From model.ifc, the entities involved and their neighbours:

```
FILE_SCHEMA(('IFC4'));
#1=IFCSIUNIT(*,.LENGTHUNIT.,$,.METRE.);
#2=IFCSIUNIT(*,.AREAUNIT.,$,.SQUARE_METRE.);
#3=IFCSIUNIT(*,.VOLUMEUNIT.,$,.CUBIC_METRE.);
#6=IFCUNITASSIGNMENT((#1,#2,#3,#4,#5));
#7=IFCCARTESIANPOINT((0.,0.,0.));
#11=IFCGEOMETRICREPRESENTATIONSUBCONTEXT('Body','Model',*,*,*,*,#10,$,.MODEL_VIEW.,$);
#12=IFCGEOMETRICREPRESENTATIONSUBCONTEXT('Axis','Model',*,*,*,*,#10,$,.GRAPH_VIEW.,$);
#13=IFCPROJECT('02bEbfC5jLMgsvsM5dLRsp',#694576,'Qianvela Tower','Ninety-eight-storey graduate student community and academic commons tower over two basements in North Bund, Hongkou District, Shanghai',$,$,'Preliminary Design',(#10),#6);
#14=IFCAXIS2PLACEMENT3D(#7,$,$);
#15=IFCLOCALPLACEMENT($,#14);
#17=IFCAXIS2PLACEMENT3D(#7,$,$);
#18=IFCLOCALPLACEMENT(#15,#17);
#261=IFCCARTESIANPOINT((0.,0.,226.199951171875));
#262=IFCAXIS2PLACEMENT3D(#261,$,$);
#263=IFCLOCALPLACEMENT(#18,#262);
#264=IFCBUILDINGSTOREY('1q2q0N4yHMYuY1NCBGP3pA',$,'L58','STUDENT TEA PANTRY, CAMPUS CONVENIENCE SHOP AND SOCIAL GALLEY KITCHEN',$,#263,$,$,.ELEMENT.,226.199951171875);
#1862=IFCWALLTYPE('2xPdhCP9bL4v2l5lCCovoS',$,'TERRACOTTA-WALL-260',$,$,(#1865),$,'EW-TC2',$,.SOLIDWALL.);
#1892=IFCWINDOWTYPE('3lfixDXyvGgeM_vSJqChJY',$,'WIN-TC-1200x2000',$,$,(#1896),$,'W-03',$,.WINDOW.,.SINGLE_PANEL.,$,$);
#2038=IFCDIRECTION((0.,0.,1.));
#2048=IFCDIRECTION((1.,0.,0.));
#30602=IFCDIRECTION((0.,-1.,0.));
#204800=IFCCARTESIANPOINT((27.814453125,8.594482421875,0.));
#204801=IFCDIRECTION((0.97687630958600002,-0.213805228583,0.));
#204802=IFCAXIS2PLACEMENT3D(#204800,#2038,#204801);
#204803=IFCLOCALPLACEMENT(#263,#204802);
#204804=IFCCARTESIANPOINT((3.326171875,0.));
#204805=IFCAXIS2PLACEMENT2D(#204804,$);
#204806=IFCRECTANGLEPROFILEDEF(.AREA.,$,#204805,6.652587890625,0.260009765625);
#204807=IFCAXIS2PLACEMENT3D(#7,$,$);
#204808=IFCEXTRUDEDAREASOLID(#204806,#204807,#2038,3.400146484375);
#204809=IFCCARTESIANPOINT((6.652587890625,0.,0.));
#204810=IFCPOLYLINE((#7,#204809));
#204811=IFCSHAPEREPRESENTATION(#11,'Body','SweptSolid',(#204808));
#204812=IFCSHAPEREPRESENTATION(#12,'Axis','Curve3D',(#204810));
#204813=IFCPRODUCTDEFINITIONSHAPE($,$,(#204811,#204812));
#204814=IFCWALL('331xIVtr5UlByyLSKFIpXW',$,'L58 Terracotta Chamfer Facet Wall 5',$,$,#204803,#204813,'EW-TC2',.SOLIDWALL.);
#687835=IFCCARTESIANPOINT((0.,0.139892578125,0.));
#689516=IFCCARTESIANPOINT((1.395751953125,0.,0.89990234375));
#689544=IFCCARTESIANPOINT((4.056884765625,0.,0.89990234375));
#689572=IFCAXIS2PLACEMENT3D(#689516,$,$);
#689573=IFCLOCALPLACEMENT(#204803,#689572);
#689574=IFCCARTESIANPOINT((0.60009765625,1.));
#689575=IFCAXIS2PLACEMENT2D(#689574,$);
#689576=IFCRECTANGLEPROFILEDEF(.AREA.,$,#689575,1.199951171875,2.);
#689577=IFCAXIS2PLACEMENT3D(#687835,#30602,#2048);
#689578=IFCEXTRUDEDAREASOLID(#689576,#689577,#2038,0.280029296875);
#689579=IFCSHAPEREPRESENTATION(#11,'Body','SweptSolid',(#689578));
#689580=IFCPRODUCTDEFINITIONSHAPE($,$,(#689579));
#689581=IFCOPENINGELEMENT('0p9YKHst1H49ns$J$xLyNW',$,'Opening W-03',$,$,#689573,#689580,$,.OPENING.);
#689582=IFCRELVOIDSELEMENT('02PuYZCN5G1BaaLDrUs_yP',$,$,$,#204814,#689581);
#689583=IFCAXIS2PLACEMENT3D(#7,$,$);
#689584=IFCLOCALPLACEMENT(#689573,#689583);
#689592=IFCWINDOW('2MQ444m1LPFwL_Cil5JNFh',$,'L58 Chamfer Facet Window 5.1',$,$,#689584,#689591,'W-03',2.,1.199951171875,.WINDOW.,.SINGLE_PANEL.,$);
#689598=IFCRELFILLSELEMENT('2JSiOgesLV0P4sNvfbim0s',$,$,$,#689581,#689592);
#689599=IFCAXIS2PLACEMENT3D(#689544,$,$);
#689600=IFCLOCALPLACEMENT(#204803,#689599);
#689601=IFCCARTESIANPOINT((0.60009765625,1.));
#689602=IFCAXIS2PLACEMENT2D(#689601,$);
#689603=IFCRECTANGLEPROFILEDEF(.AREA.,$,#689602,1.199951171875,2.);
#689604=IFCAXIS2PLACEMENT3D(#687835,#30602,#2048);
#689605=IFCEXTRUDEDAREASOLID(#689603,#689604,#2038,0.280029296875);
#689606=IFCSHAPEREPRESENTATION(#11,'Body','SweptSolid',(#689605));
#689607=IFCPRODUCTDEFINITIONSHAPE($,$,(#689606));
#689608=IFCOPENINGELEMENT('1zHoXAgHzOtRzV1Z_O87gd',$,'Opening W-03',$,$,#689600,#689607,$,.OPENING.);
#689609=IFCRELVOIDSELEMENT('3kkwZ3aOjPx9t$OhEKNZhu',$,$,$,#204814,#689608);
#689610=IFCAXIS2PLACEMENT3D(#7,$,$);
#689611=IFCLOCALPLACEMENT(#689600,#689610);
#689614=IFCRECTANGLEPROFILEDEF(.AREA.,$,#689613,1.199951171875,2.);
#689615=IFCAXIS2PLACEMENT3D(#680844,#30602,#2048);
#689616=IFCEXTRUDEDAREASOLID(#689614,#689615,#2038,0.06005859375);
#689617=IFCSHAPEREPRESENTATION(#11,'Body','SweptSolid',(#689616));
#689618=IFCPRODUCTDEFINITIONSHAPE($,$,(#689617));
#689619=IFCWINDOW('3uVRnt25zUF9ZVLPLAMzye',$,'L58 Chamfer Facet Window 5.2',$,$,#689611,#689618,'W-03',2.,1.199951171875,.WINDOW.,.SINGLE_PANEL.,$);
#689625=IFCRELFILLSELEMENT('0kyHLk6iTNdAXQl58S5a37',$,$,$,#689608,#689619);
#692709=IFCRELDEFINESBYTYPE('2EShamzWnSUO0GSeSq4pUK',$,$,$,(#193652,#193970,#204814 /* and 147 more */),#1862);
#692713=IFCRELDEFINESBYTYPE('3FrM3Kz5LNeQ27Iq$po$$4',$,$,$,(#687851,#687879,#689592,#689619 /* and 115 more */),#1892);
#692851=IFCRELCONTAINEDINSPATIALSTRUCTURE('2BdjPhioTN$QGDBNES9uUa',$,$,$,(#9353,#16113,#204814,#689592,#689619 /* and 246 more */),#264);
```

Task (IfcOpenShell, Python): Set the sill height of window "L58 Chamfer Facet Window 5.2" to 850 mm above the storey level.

```python
import numpy as np
import ifcopenshell
import ifcopenshell.api.geometry
import ifcopenshell.geom
import ifcopenshell.util.element
import ifcopenshell.util.placement
import ifcopenshell.util.shape
import ifcopenshell.util.unit

model = ifcopenshell.open("model.ifc")
unit_scale = ifcopenshell.util.unit.calculate_unit_scale(model)

window = model.by_guid("3uVRnt25zUF9ZVLPLAMzye")
opening = window.FillsVoids[0].RelatingOpeningElement
storey = ifcopenshell.util.element.get_container(window, ifc_class="IfcBuildingStorey")
level = ifcopenshell.util.placement.get_local_placement(storey.ObjectPlacement)[2, 3]

# The opening's origin need not be at the sill, so measure its lowest point.
shape = ifcopenshell.geom.create_shape(ifcopenshell.geom.settings(), opening)
bottom = ifcopenshell.util.shape.get_shape_bottom_elevation(shape, shape.geometry) / unit_scale
dz = level + 0.85 - bottom

shift = np.array([0.0, 0.0, dz])
# The window is placed relative to its opening, so it follows when the opening moves.
matrix = ifcopenshell.util.placement.get_local_placement(opening.ObjectPlacement)
matrix[:3, 3] += shift
ifcopenshell.api.geometry.edit_object_placement(
    model, product=opening, matrix=matrix, is_si=False, should_transform_children=True
)

print(f"moved by {dz * unit_scale:+.3f} m")

model.write("model_rev.ifc")
```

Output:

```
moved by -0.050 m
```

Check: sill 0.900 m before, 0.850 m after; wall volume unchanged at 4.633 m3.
